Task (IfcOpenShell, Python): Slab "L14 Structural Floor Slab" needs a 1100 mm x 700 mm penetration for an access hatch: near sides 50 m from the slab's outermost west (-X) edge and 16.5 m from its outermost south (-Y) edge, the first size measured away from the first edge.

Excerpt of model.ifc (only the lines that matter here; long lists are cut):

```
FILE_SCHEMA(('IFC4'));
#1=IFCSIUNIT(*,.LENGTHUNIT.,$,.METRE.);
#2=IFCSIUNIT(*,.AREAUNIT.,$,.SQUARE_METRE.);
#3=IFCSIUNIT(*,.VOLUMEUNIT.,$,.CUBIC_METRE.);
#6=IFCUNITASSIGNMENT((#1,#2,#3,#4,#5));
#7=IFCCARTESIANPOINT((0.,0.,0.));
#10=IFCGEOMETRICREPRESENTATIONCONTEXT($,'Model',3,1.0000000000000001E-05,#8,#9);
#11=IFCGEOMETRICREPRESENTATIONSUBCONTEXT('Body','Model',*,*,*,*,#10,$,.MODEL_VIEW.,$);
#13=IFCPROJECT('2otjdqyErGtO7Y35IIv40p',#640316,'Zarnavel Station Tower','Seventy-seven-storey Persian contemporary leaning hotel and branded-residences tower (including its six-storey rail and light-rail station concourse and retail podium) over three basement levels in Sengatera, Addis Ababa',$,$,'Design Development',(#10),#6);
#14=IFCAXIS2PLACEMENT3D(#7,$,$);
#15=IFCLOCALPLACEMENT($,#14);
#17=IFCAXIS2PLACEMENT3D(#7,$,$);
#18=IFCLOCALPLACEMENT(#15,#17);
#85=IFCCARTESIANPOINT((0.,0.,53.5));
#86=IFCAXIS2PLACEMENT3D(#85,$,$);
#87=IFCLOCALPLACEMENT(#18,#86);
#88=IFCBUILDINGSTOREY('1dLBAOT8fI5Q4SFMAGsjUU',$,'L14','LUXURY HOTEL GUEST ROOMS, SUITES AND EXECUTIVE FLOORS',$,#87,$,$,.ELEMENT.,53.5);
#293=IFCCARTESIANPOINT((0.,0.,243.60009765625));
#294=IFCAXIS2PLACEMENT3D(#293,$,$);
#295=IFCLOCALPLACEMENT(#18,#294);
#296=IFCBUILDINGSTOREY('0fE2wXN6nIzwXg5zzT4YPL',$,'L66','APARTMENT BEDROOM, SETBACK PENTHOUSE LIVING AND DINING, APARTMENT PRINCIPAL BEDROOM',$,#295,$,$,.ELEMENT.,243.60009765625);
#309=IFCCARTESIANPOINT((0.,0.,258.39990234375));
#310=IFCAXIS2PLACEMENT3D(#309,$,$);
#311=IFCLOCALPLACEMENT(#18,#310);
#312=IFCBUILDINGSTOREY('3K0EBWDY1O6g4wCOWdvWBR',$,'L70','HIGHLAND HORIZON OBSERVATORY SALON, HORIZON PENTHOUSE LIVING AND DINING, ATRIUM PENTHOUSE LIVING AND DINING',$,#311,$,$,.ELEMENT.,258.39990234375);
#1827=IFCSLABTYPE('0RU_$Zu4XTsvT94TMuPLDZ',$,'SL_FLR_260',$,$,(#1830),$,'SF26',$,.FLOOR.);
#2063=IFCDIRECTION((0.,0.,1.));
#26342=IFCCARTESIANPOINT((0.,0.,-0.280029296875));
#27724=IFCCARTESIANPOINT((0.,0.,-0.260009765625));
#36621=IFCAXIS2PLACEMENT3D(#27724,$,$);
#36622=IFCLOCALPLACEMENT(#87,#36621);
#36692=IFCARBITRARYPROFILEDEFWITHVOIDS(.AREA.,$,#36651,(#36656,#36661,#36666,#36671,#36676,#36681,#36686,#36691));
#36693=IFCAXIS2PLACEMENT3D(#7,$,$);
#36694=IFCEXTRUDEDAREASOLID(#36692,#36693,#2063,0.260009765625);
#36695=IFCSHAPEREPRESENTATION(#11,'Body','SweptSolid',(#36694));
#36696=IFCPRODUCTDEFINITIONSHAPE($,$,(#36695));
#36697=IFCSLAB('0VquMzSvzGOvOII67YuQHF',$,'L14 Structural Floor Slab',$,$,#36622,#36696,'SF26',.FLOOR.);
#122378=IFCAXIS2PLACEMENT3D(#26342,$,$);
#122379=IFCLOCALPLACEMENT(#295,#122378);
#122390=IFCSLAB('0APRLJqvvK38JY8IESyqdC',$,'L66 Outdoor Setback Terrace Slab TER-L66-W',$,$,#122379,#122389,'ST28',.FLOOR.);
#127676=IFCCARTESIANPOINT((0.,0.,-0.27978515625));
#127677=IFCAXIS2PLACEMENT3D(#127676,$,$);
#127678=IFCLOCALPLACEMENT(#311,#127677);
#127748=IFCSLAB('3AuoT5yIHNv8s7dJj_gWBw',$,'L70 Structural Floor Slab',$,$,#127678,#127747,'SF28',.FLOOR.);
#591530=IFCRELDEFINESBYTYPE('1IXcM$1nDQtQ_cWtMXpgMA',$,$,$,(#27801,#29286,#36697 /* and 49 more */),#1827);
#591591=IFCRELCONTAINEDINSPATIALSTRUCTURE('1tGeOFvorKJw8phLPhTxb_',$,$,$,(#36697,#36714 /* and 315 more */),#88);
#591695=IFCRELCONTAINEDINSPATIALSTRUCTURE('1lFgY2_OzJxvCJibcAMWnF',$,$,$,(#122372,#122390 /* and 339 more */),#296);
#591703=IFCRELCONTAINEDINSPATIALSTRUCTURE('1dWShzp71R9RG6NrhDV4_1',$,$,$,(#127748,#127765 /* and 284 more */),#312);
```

```python
import numpy as np
import ifcopenshell
import ifcopenshell.api.feature
import ifcopenshell.api.geometry
import ifcopenshell.api.root
import ifcopenshell.geom
import ifcopenshell.util.placement
import ifcopenshell.util.representation
import ifcopenshell.util.shape
import ifcopenshell.util.unit

model = ifcopenshell.open("model.ifc")
unit_scale = ifcopenshell.util.unit.calculate_unit_scale(model)
settings = ifcopenshell.geom.settings()


def volume(element):
    """Net volume in cubic metres, openings subtracted."""
    shape = ifcopenshell.geom.create_shape(settings, element)
    return ifcopenshell.util.shape.get_volume(shape.geometry)


slab = model.by_id(36697)
before = volume(slab)

# Extent in the slab's own axes, in metres. The edges named are its -X and -Y sides.
slab_shape = ifcopenshell.geom.create_shape(settings, slab)
vertices = ifcopenshell.util.shape.get_vertices(slab_shape.geometry)
x_min, y_min, bottom = vertices.min(axis=0)
top = vertices[:, 2].max()

opening = ifcopenshell.api.root.create_entity(model, ifc_class="IfcOpeningElement", name="Access hatch opening", predefined_type="OPENING")
context = ifcopenshell.util.representation.get_context(model, "Model", "Body", "MODEL_VIEW")
width, depth = 1.1, 0.7
outline = [(0.0, 0.0), (width, 0.0), (width, depth), (0.0, depth), (0.0, 0.0)]
# Overshoot both faces by 50 mm so the cut is clean.
shape = ifcopenshell.api.geometry.add_slab_representation(
    model, context=context, depth=top - bottom + 0.1, polyline=outline
)
ifcopenshell.api.geometry.assign_representation(model, product=opening, representation=shape)

matrix = ifcopenshell.util.placement.get_local_placement(slab.ObjectPlacement)
matrix[:, 3] = matrix @ np.append(np.array([x_min + 50, y_min + 16.5, bottom - 0.05]) / unit_scale, 1.0)
ifcopenshell.api.geometry.edit_object_placement(model, product=opening, matrix=matrix, is_si=False)
ifcopenshell.api.feature.add_feature(model, feature=opening, element=slab)

after = volume(slab)

print(f"slab volume {before:.3f} -> {after:.3f} m3")

model.write("model_edited.ifc")
```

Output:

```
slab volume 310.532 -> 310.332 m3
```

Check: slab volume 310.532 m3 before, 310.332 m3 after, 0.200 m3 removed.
